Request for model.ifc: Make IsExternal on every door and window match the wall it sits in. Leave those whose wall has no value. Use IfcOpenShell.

First a look at what the model holds.

```python
import ifcopenshell
import ifcopenshell.util.element

model = ifcopenshell.open("model.ifc")
print(model.schema)
seen = {}
for e in model.by_type("IfcDoor") + model.by_type("IfcWindow"):
    if not e.FillsVoids:
        continue
    host = e.FillsVoids[0].RelatingOpeningElement.VoidsElements[0].RelatingBuildingElement
    own = ifcopenshell.util.element.get_pset(e, f"Pset_{e.is_a()[3:].removesuffix('StandardCase')}Common", "IsExternal")
    wall = ifcopenshell.util.element.get_pset(host, "Pset_WallCommon", "IsExternal")
    seen[e.is_a(), own, wall] = seen.get((e.is_a(), own, wall), 0) + 1
for (cls, own, wall), count in sorted(seen.items(), key=str):
    print(count, cls, "IsExternal:", own, "| host wall:", wall)
```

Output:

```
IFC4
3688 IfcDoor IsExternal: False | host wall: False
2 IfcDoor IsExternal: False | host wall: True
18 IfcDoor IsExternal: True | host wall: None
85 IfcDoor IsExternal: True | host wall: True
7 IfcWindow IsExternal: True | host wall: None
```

```python
import ifcopenshell
import ifcopenshell.api.pset
import ifcopenshell.util.element

model = ifcopenshell.open("model.ifc")

count = 0
for ifc_class, pset_name in (("IfcDoor", "Pset_DoorCommon"), ("IfcWindow", "Pset_WindowCommon")):
    for e in model.by_type(ifc_class):
        if not e.FillsVoids:
            continue
        host = e.FillsVoids[0].RelatingOpeningElement.VoidsElements[0].RelatingBuildingElement
        external = ifcopenshell.util.element.get_pset(host, "Pset_WallCommon", "IsExternal")
        if external is None or ifcopenshell.util.element.get_pset(e, pset_name, "IsExternal") == external:
            continue
        pset = ifcopenshell.api.pset.add_pset(model, product=e, name=pset_name)
        ifcopenshell.api.pset.edit_pset(model, pset=pset, properties={"IsExternal": external})
        count += 1

print(count, "updated")

model.write("model-out.ifc")
```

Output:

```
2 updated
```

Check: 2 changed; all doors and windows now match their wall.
